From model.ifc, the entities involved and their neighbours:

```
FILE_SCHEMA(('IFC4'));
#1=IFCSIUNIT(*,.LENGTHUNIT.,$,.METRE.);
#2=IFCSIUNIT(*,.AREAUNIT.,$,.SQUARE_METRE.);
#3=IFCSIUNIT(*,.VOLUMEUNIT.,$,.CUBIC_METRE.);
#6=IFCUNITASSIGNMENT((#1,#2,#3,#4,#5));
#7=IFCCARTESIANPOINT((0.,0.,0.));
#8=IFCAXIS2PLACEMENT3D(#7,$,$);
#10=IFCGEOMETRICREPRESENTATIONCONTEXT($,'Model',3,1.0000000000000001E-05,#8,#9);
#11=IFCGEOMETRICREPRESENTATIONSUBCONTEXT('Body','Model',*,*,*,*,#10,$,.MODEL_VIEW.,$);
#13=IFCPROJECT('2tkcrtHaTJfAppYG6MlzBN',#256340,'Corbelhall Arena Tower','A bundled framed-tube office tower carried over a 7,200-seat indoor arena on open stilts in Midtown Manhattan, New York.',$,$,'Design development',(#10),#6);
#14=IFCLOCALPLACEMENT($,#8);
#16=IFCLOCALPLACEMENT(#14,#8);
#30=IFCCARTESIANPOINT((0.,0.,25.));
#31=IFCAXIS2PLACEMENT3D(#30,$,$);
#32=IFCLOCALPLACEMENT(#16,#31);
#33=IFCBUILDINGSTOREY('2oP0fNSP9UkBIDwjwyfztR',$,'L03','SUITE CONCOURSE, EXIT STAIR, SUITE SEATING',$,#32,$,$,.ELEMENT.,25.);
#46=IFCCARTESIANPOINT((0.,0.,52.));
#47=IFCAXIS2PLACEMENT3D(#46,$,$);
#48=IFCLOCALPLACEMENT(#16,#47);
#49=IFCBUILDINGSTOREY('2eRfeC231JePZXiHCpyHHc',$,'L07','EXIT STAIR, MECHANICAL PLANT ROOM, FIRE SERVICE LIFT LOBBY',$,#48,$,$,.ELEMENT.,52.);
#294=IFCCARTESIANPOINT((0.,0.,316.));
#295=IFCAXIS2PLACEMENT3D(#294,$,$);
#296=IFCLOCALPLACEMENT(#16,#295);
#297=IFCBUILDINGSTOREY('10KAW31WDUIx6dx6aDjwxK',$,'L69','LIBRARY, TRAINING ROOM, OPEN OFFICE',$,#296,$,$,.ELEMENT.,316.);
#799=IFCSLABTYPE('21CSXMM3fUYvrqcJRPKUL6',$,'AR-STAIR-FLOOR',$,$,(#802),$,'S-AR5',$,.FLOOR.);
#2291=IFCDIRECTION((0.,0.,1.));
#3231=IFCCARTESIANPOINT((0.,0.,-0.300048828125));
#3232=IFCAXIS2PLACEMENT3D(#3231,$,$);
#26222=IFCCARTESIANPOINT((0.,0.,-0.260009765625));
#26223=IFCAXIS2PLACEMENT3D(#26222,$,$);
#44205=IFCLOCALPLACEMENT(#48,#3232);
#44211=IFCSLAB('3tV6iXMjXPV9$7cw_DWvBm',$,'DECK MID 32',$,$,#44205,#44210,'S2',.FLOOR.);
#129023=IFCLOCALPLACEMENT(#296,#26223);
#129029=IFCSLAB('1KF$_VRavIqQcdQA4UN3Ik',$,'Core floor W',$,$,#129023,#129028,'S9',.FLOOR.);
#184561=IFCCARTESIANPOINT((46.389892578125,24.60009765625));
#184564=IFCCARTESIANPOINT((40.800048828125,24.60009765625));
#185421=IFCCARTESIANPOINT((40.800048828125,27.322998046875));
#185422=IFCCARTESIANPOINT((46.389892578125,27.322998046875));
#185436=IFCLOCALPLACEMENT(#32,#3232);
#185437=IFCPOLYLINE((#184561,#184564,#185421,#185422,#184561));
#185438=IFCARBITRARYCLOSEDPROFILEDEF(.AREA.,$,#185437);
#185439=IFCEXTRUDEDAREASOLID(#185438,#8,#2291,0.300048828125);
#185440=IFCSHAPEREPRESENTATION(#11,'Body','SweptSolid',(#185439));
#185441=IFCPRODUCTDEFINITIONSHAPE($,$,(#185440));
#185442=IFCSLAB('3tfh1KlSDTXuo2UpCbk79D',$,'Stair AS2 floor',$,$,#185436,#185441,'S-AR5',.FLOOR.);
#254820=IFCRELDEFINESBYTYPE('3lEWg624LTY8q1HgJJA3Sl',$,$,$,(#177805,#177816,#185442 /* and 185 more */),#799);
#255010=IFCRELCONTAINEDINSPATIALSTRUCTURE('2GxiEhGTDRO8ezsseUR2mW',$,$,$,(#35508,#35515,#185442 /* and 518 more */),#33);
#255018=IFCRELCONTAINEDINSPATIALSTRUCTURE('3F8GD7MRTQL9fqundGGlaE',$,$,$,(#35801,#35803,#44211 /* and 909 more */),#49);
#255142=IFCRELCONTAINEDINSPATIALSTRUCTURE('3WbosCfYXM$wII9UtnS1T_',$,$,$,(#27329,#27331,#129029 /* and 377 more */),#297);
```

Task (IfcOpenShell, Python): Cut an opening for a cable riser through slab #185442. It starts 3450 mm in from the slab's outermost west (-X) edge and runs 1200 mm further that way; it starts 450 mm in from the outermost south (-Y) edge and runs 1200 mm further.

```python
import numpy as np
import ifcopenshell
import ifcopenshell.api.feature
import ifcopenshell.api.geometry
import ifcopenshell.api.root
import ifcopenshell.geom
import ifcopenshell.util.placement
import ifcopenshell.util.representation
import ifcopenshell.util.shape
import ifcopenshell.util.unit

model = ifcopenshell.open("model.ifc")
unit_scale = ifcopenshell.util.unit.calculate_unit_scale(model)
settings = ifcopenshell.geom.settings()


def volume(element):
    """Net volume in cubic metres, openings subtracted."""
    shape = ifcopenshell.geom.create_shape(settings, element)
    return ifcopenshell.util.shape.get_volume(shape.geometry)


slab = model.by_guid("3tfh1KlSDTXuo2UpCbk79D")
before = volume(slab)

# Extent in the slab's own axes, in metres. The edges named are its -X and -Y sides.
slab_shape = ifcopenshell.geom.create_shape(settings, slab)
vertices = ifcopenshell.util.shape.get_vertices(slab_shape.geometry)
x_min, y_min, bottom = vertices.min(axis=0)
top = vertices[:, 2].max()

opening = ifcopenshell.api.root.create_entity(model, ifc_class="IfcOpeningElement", name="Cable riser opening", predefined_type="OPENING")
context = ifcopenshell.util.representation.get_context(model, "Model", "Body", "MODEL_VIEW")
width, depth = 1.2, 1.2
outline = [(0.0, 0.0), (width, 0.0), (width, depth), (0.0, depth), (0.0, 0.0)]
# Overshoot both faces by 50 mm so the cut is clean.
shape = ifcopenshell.api.geometry.add_slab_representation(
    model, context=context, depth=top - bottom + 0.1, polyline=outline
)
ifcopenshell.api.geometry.assign_representation(model, product=opening, representation=shape)

matrix = ifcopenshell.util.placement.get_local_placement(slab.ObjectPlacement)
matrix[:, 3] = matrix @ np.append(np.array([x_min + 3.45, y_min + 0.45, bottom - 0.05]) / unit_scale, 1.0)
ifcopenshell.api.geometry.edit_object_placement(model, product=opening, matrix=matrix, is_si=False)
ifcopenshell.api.feature.add_feature(model, feature=opening, element=slab)

after = volume(slab)

print(f"slab volume {before:.3f} -> {after:.3f} m3")

model.write("model-out.ifc")
```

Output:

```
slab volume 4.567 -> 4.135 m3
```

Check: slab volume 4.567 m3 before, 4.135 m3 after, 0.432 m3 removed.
